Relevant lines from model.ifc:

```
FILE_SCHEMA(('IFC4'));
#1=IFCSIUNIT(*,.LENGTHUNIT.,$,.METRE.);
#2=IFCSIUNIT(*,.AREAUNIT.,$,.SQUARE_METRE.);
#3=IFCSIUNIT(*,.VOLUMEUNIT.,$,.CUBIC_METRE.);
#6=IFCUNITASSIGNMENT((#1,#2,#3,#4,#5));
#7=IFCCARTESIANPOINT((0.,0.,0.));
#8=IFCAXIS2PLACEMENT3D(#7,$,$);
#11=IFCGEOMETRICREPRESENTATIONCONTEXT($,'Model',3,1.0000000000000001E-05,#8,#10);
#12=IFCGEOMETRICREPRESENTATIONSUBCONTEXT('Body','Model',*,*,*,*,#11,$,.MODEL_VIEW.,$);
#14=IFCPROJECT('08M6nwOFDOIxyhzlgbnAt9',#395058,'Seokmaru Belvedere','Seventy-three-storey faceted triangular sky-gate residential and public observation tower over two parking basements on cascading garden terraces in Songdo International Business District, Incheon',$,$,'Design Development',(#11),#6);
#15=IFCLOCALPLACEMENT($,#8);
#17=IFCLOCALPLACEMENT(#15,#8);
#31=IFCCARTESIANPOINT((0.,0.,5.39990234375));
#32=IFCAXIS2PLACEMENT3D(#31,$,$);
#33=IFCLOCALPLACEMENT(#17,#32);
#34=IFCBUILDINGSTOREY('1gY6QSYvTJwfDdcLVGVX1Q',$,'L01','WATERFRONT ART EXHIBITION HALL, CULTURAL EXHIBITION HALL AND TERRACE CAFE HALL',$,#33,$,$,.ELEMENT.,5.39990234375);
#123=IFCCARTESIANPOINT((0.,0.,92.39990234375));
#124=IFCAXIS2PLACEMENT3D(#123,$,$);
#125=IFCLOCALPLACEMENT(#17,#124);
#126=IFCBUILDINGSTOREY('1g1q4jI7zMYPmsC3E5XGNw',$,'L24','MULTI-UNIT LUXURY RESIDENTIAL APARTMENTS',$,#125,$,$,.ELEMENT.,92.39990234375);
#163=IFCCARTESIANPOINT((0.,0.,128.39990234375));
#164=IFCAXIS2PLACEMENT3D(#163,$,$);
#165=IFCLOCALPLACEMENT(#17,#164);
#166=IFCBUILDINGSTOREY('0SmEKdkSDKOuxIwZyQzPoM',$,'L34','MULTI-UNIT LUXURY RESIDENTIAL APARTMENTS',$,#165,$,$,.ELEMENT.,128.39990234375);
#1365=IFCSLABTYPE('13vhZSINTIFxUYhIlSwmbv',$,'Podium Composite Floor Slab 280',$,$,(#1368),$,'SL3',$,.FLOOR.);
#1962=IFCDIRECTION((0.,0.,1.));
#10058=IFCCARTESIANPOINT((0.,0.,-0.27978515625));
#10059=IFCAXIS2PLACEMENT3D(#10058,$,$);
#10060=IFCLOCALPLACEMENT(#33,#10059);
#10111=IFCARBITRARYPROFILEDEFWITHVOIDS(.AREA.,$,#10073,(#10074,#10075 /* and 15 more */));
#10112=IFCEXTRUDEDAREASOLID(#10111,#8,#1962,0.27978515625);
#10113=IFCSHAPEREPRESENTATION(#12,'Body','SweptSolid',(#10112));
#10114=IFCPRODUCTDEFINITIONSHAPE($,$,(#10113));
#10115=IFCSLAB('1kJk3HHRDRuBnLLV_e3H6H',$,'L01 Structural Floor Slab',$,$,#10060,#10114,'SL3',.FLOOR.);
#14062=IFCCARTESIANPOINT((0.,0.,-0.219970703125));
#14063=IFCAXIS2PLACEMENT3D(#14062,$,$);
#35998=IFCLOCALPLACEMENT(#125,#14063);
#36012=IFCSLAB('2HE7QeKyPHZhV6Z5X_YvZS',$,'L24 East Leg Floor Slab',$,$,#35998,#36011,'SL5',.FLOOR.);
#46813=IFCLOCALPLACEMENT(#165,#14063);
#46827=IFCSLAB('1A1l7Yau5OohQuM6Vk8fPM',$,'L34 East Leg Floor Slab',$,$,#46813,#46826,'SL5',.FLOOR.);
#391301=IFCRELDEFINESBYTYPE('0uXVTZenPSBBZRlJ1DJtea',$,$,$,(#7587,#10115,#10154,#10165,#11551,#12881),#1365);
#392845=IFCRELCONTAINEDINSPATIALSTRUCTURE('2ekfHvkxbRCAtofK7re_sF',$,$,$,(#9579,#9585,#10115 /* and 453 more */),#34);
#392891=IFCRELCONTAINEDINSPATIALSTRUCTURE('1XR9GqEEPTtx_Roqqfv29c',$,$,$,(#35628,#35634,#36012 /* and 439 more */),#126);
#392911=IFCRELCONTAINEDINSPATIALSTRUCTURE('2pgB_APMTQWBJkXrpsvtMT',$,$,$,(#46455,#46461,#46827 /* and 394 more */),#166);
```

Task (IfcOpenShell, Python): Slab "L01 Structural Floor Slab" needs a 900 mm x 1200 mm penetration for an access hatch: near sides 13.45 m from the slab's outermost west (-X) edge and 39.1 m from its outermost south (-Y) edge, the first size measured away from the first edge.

```python
import numpy as np
import ifcopenshell
import ifcopenshell.api.feature
import ifcopenshell.api.geometry
import ifcopenshell.api.root
import ifcopenshell.geom
import ifcopenshell.util.placement
import ifcopenshell.util.representation
import ifcopenshell.util.shape
import ifcopenshell.util.unit

model = ifcopenshell.open("model.ifc")
unit_scale = ifcopenshell.util.unit.calculate_unit_scale(model)
settings = ifcopenshell.geom.settings()


def volume(element):
    """Net volume in cubic metres, openings subtracted."""
    shape = ifcopenshell.geom.create_shape(settings, element)
    return ifcopenshell.util.shape.get_volume(shape.geometry)


slab = model.by_guid("1kJk3HHRDRuBnLLV_e3H6H")
before = volume(slab)

# Extent in the slab's own axes, in metres. The edges named are its -X and -Y sides.
slab_shape = ifcopenshell.geom.create_shape(settings, slab)
vertices = ifcopenshell.util.shape.get_vertices(slab_shape.geometry)
x_min, y_min, bottom = vertices.min(axis=0)
top = vertices[:, 2].max()

opening = ifcopenshell.api.root.create_entity(model, ifc_class="IfcOpeningElement", name="Access hatch opening", predefined_type="OPENING")
context = ifcopenshell.util.representation.get_context(model, "Model", "Body", "MODEL_VIEW")
width, depth = 0.9, 1.2
outline = [(0.0, 0.0), (width, 0.0), (width, depth), (0.0, depth), (0.0, 0.0)]
# Overshoot both faces by 50 mm so the cut is clean.
shape = ifcopenshell.api.geometry.add_slab_representation(
    model, context=context, depth=top - bottom + 0.1, polyline=outline
)
ifcopenshell.api.geometry.assign_representation(model, product=opening, representation=shape)

matrix = ifcopenshell.util.placement.get_local_placement(slab.ObjectPlacement)
matrix[:, 3] = matrix @ np.append(np.array([x_min + 13.45, y_min + 39.1, bottom - 0.05]) / unit_scale, 1.0)
ifcopenshell.api.geometry.edit_object_placement(model, product=opening, matrix=matrix, is_si=False)
ifcopenshell.api.feature.add_feature(model, feature=opening, element=slab)

after = volume(slab)

print(f"slab volume {before:.3f} -> {after:.3f} m3")

model.write("model_v2.ifc")
```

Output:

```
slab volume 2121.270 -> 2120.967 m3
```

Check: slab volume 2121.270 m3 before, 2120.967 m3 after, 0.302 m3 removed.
